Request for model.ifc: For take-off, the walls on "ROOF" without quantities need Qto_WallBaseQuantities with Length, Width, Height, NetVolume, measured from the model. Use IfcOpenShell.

First a look at what the model holds.

```python
import ifcopenshell
import ifcopenshell.util.element
import ifcopenshell.util.unit

model = ifcopenshell.open("model.ifc")
print(model.schema)
for unit_type in ("LENGTHUNIT", "AREAUNIT", "VOLUMEUNIT"):
    print(unit_type, ifcopenshell.util.unit.calculate_unit_scale(model, unit_type))
storey = next(s for s in model.by_type("IfcBuildingStorey") if s.Name == "ROOF")
walls = [e for e in ifcopenshell.util.element.get_decomposition(storey) if e.is_a("IfcWall")]
for e in sorted(walls, key=lambda e: e.id()):
    print(e.id(), e.is_a(), e.Name, list(ifcopenshell.util.element.get_psets(e, qtos_only=True)), sep=" | ")
```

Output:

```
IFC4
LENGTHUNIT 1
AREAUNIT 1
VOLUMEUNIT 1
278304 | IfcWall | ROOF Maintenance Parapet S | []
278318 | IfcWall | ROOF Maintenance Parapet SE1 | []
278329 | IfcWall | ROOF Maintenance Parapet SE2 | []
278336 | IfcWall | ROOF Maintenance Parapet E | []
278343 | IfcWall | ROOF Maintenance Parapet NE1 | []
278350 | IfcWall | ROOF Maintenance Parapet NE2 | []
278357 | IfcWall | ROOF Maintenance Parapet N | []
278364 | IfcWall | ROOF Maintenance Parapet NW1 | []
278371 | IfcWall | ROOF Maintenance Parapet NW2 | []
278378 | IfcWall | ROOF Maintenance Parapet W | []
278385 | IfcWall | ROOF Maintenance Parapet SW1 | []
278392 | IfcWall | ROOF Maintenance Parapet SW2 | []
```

```python
import ifcopenshell
import ifcopenshell.api.pset
import ifcopenshell.geom
import ifcopenshell.util.element
import ifcopenshell.util.shape
import ifcopenshell.util.unit

model = ifcopenshell.open("model.ifc")
unit_scale = ifcopenshell.util.unit.calculate_unit_scale(model)
volume_scale = ifcopenshell.util.unit.calculate_unit_scale(model, "VOLUMEUNIT")
settings = ifcopenshell.geom.settings()

storey = next(s for s in model.by_type("IfcBuildingStorey") if s.Name == "ROOF")
walls = [e for e in ifcopenshell.util.element.get_decomposition(storey) if e.is_a("IfcWall")]

for e in sorted(walls, key=lambda e: e.id()):
    if ifcopenshell.util.element.get_psets(e, qtos_only=True, should_inherit=False):
        continue
    # Geometry comes back in metres, in the element's own axes.
    shape = ifcopenshell.geom.create_shape(settings, e)
    values = {
        "Length": ifcopenshell.util.shape.get_x(shape.geometry) / unit_scale,
        "Width": ifcopenshell.util.shape.get_y(shape.geometry) / unit_scale,
        "Height": ifcopenshell.util.shape.get_z(shape.geometry) / unit_scale,
        "NetVolume": ifcopenshell.util.shape.get_volume(shape.geometry) / volume_scale,
    }
    qto = ifcopenshell.api.pset.add_qto(model, product=e, name="Qto_WallBaseQuantities")
    ifcopenshell.api.pset.edit_qto(model, qto=qto, properties=values)
    print(e.id(), {k: round(v, 3) for k, v in values.items()})

model.write("model-out.ifc")
```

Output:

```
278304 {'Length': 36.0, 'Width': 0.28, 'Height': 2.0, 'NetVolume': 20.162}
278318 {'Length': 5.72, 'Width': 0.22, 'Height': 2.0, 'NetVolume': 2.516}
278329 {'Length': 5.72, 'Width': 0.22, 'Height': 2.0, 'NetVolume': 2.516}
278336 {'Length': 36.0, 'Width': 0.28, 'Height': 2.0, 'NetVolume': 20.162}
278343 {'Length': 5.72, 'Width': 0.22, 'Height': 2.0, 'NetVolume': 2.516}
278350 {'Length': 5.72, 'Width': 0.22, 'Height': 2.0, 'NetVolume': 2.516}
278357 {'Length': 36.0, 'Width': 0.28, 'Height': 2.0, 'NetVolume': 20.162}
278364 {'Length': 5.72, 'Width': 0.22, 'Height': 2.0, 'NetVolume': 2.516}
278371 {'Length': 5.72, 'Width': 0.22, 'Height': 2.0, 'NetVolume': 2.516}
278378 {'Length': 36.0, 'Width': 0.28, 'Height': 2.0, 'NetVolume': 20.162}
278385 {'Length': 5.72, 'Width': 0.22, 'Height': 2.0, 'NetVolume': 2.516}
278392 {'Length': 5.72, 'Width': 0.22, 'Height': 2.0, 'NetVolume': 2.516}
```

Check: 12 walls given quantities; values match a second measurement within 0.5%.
